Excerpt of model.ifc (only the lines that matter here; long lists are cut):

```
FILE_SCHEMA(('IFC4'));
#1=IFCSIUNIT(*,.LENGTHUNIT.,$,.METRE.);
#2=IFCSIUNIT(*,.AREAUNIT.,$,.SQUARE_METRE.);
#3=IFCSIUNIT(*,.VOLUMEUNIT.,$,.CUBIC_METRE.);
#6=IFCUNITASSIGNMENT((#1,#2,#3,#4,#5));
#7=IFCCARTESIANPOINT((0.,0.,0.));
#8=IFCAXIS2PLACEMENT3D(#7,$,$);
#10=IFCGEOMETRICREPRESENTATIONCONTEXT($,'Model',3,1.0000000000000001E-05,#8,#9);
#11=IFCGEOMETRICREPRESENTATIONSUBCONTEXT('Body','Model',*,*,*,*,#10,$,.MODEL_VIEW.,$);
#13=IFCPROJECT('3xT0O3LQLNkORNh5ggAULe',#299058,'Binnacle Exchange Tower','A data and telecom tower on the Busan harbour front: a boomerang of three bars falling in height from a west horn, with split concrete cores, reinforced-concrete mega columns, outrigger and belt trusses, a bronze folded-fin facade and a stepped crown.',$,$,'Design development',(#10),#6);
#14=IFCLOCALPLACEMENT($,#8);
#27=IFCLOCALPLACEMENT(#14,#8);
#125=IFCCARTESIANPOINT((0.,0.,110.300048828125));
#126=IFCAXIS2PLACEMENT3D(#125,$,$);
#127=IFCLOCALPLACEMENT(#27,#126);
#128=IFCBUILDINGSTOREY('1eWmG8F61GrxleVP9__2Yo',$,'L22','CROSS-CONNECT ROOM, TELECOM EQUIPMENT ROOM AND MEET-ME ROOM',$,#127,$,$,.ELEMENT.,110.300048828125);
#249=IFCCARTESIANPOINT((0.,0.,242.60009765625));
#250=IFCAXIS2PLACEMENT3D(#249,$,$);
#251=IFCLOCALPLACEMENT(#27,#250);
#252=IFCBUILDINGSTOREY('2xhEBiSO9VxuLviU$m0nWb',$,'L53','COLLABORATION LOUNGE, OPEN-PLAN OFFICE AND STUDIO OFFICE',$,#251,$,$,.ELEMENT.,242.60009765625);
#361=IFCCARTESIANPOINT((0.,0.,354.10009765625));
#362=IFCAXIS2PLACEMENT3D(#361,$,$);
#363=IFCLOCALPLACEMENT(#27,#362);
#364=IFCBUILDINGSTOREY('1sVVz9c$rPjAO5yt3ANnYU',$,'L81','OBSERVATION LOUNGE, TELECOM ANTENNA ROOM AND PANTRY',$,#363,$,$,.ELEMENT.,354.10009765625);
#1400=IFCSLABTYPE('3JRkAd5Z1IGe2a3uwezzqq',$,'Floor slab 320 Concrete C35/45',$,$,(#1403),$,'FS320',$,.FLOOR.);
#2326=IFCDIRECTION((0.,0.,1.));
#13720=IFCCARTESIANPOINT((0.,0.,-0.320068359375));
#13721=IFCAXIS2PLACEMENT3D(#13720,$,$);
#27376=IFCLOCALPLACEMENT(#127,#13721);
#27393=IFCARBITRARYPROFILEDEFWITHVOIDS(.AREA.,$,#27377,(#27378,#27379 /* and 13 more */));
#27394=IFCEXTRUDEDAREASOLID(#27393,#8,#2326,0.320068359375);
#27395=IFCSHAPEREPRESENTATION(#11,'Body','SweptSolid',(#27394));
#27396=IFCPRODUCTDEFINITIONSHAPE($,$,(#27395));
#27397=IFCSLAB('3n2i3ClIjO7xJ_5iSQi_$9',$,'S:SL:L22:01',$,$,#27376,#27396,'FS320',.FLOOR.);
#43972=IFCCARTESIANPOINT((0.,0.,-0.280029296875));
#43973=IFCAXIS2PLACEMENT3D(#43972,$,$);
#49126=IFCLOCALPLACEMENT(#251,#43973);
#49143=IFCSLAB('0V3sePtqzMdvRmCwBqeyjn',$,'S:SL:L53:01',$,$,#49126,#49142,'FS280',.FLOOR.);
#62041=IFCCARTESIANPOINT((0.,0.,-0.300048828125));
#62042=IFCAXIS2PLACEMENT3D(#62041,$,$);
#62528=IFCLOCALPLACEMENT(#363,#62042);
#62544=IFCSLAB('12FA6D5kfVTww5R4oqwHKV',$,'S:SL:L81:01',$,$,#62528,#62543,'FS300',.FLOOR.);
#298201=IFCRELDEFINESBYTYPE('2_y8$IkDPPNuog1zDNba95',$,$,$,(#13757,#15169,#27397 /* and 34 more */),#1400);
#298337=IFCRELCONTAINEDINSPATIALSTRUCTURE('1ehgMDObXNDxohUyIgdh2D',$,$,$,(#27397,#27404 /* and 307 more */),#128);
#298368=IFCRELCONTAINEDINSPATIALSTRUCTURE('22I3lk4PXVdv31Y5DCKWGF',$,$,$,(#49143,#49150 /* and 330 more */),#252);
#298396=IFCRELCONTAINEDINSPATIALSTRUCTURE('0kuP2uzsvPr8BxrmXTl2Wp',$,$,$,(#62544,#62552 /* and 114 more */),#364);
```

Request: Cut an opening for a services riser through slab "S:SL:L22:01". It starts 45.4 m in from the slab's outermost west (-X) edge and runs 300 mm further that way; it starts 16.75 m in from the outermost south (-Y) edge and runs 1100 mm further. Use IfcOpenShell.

```python
import numpy as np
import ifcopenshell
import ifcopenshell.api.feature
import ifcopenshell.api.geometry
import ifcopenshell.api.root
import ifcopenshell.geom
import ifcopenshell.util.placement
import ifcopenshell.util.representation
import ifcopenshell.util.shape
import ifcopenshell.util.unit

model = ifcopenshell.open("model.ifc")
unit_scale = ifcopenshell.util.unit.calculate_unit_scale(model)
settings = ifcopenshell.geom.settings()


def volume(element):
    """Net volume in cubic metres, openings subtracted."""
    shape = ifcopenshell.geom.create_shape(settings, element)
    return ifcopenshell.util.shape.get_volume(shape.geometry)


slab = model.by_id(27397)
before = volume(slab)

# Extent in the slab's own axes, in metres. The edges named are its -X and -Y sides.
slab_shape = ifcopenshell.geom.create_shape(settings, slab)
vertices = ifcopenshell.util.shape.get_vertices(slab_shape.geometry)
x_min, y_min, bottom = vertices.min(axis=0)
top = vertices[:, 2].max()

opening = ifcopenshell.api.root.create_entity(model, ifc_class="IfcOpeningElement", name="Services riser opening", predefined_type="OPENING")
context = ifcopenshell.util.representation.get_context(model, "Model", "Body", "MODEL_VIEW")
width, depth = 0.3, 1.1
outline = [(0.0, 0.0), (width, 0.0), (width, depth), (0.0, depth), (0.0, 0.0)]
# Overshoot both faces by 50 mm so the cut is clean.
shape = ifcopenshell.api.geometry.add_slab_representation(
    model, context=context, depth=top - bottom + 0.1, polyline=outline
)
ifcopenshell.api.geometry.assign_representation(model, product=opening, representation=shape)

matrix = ifcopenshell.util.placement.get_local_placement(slab.ObjectPlacement)
matrix[:, 3] = matrix @ np.append(np.array([x_min + 45.4, y_min + 16.75, bottom - 0.05]) / unit_scale, 1.0)
ifcopenshell.api.geometry.edit_object_placement(model, product=opening, matrix=matrix, is_si=False)
ifcopenshell.api.feature.add_feature(model, feature=opening, element=slab)

after = volume(slab)

print(f"slab volume {before:.3f} -> {after:.3f} m3")

model.write("model_v2.ifc")
```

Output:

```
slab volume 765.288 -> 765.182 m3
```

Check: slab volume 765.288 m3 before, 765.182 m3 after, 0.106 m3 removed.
